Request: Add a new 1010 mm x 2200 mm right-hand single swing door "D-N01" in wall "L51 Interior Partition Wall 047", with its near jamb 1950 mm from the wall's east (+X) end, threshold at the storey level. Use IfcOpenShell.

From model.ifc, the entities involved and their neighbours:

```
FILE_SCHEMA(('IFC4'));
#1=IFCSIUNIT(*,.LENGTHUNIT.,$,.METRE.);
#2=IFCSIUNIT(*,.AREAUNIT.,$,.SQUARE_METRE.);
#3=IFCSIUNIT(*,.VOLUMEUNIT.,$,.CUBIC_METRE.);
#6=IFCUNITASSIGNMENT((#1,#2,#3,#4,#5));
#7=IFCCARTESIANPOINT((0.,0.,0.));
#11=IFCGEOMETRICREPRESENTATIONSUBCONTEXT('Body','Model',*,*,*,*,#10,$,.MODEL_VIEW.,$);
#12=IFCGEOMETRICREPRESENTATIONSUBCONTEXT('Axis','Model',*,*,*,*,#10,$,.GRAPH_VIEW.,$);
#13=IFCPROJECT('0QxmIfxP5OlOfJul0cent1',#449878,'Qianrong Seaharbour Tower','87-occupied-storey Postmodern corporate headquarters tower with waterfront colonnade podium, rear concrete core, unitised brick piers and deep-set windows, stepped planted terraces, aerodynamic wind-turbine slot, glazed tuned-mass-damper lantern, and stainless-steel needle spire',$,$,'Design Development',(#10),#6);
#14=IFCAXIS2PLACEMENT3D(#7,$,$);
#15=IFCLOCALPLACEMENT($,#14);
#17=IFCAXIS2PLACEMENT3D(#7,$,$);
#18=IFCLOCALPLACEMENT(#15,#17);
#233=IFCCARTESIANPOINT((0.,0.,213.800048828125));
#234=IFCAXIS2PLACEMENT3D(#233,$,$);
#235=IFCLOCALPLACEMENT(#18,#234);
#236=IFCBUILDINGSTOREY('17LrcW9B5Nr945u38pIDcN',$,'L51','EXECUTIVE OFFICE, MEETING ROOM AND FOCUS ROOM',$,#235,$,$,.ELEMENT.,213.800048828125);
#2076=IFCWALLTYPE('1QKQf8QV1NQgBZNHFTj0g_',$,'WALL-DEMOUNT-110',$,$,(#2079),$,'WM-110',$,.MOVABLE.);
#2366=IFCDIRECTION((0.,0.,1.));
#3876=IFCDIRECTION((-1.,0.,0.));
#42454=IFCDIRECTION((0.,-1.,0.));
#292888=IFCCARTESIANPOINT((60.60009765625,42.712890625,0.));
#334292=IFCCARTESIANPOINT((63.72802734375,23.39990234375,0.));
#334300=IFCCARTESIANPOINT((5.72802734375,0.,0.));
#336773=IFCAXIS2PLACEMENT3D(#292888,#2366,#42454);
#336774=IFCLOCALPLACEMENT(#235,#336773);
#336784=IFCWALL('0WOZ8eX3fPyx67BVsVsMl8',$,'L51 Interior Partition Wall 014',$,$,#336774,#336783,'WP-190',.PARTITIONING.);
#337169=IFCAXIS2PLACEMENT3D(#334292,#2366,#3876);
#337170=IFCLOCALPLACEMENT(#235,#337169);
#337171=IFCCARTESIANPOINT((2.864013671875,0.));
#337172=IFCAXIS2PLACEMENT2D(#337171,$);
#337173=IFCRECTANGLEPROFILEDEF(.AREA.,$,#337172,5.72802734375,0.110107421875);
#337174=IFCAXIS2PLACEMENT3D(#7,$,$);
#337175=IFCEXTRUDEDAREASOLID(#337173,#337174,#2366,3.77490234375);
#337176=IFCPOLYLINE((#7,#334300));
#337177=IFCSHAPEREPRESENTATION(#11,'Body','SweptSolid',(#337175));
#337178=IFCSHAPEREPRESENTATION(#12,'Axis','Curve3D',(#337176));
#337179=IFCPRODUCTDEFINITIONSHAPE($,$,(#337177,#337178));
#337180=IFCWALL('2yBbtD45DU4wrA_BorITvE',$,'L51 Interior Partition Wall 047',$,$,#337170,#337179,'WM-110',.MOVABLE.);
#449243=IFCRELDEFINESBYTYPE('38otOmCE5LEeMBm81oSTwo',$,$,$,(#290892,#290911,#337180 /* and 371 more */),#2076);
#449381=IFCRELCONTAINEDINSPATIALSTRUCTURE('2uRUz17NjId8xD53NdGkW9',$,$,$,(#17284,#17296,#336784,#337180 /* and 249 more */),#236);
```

```python
import numpy as np
import ifcopenshell
import ifcopenshell.api.feature
import ifcopenshell.api.geometry
import ifcopenshell.api.root
import ifcopenshell.api.spatial
import ifcopenshell.geom
import ifcopenshell.util.element
import ifcopenshell.util.placement
import ifcopenshell.util.representation
import ifcopenshell.util.shape
import ifcopenshell.util.unit

model = ifcopenshell.open("model.ifc")
unit_scale = ifcopenshell.util.unit.calculate_unit_scale(model)
settings = ifcopenshell.geom.settings()


def volume(element):
    """Net volume in cubic metres, openings subtracted."""
    shape = ifcopenshell.geom.create_shape(settings, element)
    return ifcopenshell.util.shape.get_volume(shape.geometry)


wall = model.by_guid("2yBbtD45DU4wrA_BorITvE")
storey = ifcopenshell.util.element.get_container(wall, ifc_class="IfcBuildingStorey")
context = ifcopenshell.util.representation.get_context(model, "Model", "Body", "MODEL_VIEW")
before = volume(wall)

width, height, from_end, sill = 1.01, 2.2, 1.95, 0.0  # metres

# The wall runs along its own X axis, and the end named is its -X end.
wall_shape = ifcopenshell.geom.create_shape(settings, wall)
x, y, z = ifcopenshell.util.shape.get_vertices(wall_shape.geometry).T
start = x.min() + from_end
face, thickness = float(y.min()), float(y.max() - y.min())
wall_matrix = ifcopenshell.util.placement.get_local_placement(wall.ObjectPlacement)
level = ifcopenshell.util.placement.get_local_placement(storey.ObjectPlacement)[2, 3]


def in_wall(x, y):
    """Placement at x, y metres in the wall's axes, at sill height."""
    matrix = wall_matrix.copy()
    matrix[:, 3] = wall_matrix @ np.array([x / unit_scale, y / unit_scale, 0.0, 1.0])
    matrix[2, 3] = level + sill / unit_scale
    return matrix


# Opening: a box that overshoots both wall faces by 50 mm.
opening = ifcopenshell.api.root.create_entity(model, ifc_class="IfcOpeningElement", predefined_type="OPENING")
box = ifcopenshell.api.geometry.add_wall_representation(
    model, context=context, length=width, height=height, thickness=thickness + 0.1
)
ifcopenshell.api.geometry.assign_representation(model, product=opening, representation=box)
ifcopenshell.api.geometry.edit_object_placement(model, product=opening, matrix=in_wall(start, face - 0.05), is_si=False)
ifcopenshell.api.feature.add_feature(model, feature=opening, element=wall)

door = ifcopenshell.api.root.create_entity(model, ifc_class="IfcDoor", name="D-N01", predefined_type="DOOR")
door.OverallWidth, door.OverallHeight = width / unit_scale, height / unit_scale
door.OperationType = "SINGLE_SWING_RIGHT"
body = ifcopenshell.api.geometry.add_door_representation(
    model,
    context=context,
    overall_width=door.OverallWidth,
    overall_height=door.OverallHeight,
    operation_type="SINGLE_SWING_RIGHT",
    lining_properties={"LiningDepth": thickness / unit_scale, "ThresholdDepth": thickness / unit_scale},
)
ifcopenshell.api.geometry.assign_representation(model, product=door, representation=body)
ifcopenshell.api.spatial.assign_container(model, products=[door], relating_structure=storey)
ifcopenshell.api.feature.add_filling(model, opening=opening, element=door)

# The lining spans the wall, so the door starts at the wall face.
ifcopenshell.api.geometry.edit_object_placement(model, product=door, matrix=in_wall(start, face), is_si=False)

after = volume(wall)

print(f"wall volume {before:.3f} -> {after:.3f} m3")

model.write("model_v2.ifc")
```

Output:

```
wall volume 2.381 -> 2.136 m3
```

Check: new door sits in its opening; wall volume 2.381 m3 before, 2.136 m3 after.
